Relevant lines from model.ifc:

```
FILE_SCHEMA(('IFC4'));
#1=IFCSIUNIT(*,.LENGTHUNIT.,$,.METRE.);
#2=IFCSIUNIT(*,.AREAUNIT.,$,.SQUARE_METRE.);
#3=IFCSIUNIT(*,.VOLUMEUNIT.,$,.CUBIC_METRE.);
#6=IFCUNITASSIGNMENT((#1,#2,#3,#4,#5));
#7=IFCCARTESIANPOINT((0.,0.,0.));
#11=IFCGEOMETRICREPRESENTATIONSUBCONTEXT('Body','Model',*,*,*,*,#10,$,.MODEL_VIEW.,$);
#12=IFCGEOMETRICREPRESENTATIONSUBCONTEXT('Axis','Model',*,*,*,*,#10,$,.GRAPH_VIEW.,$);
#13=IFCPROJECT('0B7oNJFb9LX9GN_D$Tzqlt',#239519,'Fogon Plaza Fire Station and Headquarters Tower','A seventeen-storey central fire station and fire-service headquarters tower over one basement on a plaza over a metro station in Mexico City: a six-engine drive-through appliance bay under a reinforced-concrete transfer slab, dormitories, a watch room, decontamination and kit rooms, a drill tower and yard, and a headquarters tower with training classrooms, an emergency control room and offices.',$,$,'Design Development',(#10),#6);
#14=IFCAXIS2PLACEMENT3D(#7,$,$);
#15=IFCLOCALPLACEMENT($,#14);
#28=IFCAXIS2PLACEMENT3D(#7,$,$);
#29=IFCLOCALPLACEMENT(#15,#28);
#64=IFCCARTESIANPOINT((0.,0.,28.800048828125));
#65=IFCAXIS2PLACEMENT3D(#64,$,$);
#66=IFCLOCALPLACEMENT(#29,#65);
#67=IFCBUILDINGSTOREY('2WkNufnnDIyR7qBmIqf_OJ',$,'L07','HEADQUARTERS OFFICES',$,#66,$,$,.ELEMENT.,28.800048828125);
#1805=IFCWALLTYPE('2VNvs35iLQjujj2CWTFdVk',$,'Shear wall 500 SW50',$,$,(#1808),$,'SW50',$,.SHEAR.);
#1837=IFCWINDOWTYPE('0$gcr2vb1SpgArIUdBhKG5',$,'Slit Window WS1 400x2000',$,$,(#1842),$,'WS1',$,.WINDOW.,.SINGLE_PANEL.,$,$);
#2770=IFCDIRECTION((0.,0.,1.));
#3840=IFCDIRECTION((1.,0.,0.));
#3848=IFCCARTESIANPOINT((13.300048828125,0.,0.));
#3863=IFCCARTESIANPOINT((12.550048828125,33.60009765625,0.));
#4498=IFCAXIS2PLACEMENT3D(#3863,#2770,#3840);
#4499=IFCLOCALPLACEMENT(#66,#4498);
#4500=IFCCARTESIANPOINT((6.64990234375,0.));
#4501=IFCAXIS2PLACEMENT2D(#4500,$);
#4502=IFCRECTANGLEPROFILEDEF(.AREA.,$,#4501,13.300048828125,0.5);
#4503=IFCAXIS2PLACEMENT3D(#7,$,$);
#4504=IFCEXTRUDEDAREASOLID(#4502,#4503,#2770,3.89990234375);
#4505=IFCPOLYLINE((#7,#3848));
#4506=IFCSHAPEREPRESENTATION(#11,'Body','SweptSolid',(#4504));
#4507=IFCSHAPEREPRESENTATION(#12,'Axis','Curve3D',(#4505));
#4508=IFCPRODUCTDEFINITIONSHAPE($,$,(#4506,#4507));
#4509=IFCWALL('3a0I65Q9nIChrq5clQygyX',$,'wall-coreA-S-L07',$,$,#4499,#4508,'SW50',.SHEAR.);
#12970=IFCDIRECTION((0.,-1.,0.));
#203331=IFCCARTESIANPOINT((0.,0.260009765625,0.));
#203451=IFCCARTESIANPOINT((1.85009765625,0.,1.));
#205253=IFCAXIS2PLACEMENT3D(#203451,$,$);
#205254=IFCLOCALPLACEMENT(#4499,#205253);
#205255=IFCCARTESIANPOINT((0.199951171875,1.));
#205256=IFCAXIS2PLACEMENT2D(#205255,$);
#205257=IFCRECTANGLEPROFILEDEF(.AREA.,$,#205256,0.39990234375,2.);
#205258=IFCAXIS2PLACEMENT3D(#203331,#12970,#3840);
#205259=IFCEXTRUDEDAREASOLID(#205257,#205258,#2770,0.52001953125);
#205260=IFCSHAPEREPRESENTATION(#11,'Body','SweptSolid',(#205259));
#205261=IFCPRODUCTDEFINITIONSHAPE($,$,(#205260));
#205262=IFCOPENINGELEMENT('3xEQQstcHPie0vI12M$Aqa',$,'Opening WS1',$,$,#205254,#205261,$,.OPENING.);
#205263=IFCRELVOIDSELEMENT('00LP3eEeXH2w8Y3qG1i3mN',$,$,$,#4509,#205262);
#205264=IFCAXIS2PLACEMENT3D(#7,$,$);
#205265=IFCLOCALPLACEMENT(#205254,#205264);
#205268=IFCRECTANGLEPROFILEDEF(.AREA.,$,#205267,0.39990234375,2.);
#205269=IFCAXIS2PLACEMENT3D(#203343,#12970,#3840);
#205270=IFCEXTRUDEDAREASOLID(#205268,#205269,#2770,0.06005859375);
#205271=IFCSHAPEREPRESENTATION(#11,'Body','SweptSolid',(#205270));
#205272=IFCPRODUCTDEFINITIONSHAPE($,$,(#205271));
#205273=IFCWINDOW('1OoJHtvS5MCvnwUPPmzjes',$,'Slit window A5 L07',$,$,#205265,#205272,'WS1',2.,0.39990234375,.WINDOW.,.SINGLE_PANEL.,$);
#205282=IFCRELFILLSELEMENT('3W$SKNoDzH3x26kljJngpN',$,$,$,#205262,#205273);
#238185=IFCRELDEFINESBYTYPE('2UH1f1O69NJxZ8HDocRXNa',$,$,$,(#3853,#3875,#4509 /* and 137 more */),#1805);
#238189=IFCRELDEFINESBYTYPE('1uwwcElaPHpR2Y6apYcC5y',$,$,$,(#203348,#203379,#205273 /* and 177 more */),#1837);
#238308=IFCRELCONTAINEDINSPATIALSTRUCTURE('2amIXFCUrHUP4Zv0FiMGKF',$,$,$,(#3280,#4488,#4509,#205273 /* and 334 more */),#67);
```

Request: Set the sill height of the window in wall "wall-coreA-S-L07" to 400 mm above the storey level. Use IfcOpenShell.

```python
import numpy as np
import ifcopenshell
import ifcopenshell.api.geometry
import ifcopenshell.geom
import ifcopenshell.util.element
import ifcopenshell.util.placement
import ifcopenshell.util.shape
import ifcopenshell.util.unit

model = ifcopenshell.open("model.ifc")
unit_scale = ifcopenshell.util.unit.calculate_unit_scale(model)

window = model.by_guid("1OoJHtvS5MCvnwUPPmzjes")
opening = window.FillsVoids[0].RelatingOpeningElement
storey = ifcopenshell.util.element.get_container(window, ifc_class="IfcBuildingStorey")
level = ifcopenshell.util.placement.get_local_placement(storey.ObjectPlacement)[2, 3]

# The opening's origin need not be at the sill, so measure its lowest point.
shape = ifcopenshell.geom.create_shape(ifcopenshell.geom.settings(), opening)
bottom = ifcopenshell.util.shape.get_shape_bottom_elevation(shape, shape.geometry) / unit_scale
dz = level + 0.4 / unit_scale - bottom

shift = np.array([0.0, 0.0, dz])
# The window is placed relative to its opening, so it follows when the opening moves.
matrix = ifcopenshell.util.placement.get_local_placement(opening.ObjectPlacement)
matrix[:3, 3] += shift
ifcopenshell.api.geometry.edit_object_placement(
    model, product=opening, matrix=matrix, is_si=False, should_transform_children=True
)

print(f"moved by {dz * unit_scale:+.3f} m")

model.write("model_v2.ifc")
```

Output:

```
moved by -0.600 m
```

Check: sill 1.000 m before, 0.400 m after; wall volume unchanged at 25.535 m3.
